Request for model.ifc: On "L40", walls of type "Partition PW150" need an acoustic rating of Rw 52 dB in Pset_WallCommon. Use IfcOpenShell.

First a look at what the model holds.

```python
import ifcopenshell
import ifcopenshell.util.element

model = ifcopenshell.open("model.ifc")
print(model.schema)
storey = next(s for s in model.by_type("IfcBuildingStorey") if s.Name == "L40")
walls = [e for e in ifcopenshell.util.element.get_decomposition(storey) if e.is_a("IfcWall")]
seen = {}
for e in walls:
    element_type = ifcopenshell.util.element.get_type(e)
    key = (element_type.Name if element_type != e and element_type else None, ifcopenshell.util.element.get_pset(e, "Pset_WallCommon", "AcousticRating"))
    seen[key] = seen.get(key, 0) + 1
for (name, value), count in sorted(seen.items(), key=str):
    print(count, "x", name, "|", value)
```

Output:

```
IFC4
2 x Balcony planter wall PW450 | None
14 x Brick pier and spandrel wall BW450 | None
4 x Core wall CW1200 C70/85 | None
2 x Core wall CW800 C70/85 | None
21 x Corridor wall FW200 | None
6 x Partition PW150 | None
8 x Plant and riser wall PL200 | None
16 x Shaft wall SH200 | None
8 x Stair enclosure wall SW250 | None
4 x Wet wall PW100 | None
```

```python
import ifcopenshell
import ifcopenshell.api.pset
import ifcopenshell.util.element

model = ifcopenshell.open("model.ifc")

storey = next(s for s in model.by_type("IfcBuildingStorey") if s.Name == "L40")
walls = [e for e in ifcopenshell.util.element.get_decomposition(storey) if e.is_a("IfcWall")]

count = 0
for e in walls:
    element_type = ifcopenshell.util.element.get_type(e)
    if element_type in (None, e) or element_type.Name != "Partition PW150":
        continue
    found = ifcopenshell.util.element.get_pset(e, "Pset_WallCommon", should_inherit=False)
    if found:
        pset = model.by_id(found["id"])
        if len(ifcopenshell.util.element.get_elements_by_pset(pset)) > 1:
            pset = ifcopenshell.api.pset.unshare_pset(model, products=[e], pset=pset)[0]
    else:
        pset = ifcopenshell.api.pset.add_pset(model, product=e, name="Pset_WallCommon")
    ifcopenshell.api.pset.edit_pset(model, pset=pset, properties={"AcousticRating": "Rw 52 dB"})
    count += 1

print(count, "walls updated")

model.write("model_edited.ifc")
```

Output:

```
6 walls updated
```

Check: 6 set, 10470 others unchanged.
